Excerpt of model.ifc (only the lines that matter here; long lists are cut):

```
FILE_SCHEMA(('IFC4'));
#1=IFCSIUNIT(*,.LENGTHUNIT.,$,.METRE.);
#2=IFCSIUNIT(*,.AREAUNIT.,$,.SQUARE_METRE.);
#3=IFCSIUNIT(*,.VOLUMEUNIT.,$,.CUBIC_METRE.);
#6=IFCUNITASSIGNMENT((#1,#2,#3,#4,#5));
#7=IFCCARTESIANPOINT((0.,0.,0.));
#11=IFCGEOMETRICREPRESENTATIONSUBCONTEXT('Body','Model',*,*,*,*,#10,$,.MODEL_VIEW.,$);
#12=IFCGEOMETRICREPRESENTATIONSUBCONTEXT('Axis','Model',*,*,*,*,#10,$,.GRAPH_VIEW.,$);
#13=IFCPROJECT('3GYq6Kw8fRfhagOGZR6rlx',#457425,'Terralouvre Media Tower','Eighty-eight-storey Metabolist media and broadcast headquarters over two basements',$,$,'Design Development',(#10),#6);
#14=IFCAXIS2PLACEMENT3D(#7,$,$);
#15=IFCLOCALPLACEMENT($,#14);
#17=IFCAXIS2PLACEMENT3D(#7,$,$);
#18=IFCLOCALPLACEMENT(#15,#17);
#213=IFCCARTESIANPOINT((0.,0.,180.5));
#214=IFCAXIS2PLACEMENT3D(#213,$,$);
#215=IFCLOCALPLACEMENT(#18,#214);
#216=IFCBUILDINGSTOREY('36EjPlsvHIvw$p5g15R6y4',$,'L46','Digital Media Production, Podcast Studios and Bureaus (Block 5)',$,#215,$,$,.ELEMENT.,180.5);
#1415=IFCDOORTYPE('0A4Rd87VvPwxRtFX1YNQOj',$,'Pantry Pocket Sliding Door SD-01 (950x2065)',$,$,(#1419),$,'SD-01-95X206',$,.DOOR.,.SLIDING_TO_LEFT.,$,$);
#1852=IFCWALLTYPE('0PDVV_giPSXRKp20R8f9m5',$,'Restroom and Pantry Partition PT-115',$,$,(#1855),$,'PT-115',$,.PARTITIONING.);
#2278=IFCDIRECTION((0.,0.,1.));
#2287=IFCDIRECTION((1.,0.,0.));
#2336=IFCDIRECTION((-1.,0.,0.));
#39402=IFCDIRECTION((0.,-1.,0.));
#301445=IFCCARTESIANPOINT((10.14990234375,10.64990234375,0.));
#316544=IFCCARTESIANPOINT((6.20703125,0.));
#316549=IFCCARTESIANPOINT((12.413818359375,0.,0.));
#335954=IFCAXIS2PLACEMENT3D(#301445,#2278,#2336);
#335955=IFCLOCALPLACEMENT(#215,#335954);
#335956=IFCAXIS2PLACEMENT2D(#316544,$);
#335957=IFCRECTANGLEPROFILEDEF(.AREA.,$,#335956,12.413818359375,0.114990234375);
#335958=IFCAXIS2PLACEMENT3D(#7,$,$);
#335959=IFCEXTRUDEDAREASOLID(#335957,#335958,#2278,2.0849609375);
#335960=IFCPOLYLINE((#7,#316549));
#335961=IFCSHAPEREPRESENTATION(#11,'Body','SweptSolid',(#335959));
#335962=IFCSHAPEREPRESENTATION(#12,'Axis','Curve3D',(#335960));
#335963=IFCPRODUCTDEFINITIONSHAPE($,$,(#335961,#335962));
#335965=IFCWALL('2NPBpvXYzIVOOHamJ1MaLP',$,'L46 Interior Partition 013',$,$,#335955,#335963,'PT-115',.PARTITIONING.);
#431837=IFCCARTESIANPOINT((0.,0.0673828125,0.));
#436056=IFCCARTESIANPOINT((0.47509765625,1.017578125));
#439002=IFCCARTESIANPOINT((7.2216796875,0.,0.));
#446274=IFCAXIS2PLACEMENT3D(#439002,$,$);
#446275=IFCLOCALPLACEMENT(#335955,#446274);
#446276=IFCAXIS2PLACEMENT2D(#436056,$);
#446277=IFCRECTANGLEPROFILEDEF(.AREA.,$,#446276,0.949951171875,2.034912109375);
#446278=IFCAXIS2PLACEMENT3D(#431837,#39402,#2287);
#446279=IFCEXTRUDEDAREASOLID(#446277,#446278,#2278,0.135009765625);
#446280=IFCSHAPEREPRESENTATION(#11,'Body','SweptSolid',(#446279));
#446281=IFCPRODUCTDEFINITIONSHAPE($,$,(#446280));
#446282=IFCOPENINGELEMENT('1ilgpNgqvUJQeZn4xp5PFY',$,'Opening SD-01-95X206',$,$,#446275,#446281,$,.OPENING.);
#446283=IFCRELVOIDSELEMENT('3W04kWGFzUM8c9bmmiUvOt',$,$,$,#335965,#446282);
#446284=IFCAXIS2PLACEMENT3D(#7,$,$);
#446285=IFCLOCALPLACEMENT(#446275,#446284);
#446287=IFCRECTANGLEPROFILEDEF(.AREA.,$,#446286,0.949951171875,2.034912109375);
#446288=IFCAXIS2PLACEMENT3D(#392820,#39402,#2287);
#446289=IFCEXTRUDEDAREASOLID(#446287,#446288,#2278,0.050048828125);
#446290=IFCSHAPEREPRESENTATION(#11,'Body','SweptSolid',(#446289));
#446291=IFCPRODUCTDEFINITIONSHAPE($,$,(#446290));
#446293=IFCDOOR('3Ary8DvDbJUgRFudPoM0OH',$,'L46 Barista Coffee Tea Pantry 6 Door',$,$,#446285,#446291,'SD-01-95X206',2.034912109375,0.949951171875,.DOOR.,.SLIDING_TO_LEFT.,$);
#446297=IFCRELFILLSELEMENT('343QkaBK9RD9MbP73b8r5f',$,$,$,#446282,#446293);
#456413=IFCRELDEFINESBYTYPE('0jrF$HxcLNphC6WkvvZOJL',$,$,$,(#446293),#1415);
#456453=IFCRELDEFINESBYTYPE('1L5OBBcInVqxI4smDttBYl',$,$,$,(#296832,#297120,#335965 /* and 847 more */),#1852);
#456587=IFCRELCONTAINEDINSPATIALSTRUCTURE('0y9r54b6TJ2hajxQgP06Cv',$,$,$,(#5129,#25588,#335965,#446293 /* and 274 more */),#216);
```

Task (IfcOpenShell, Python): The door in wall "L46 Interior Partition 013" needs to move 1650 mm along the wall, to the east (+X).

```python
import ifcopenshell
import ifcopenshell.api.geometry
import ifcopenshell.util.placement
import ifcopenshell.util.unit

model = ifcopenshell.open("model.ifc")
unit_scale = ifcopenshell.util.unit.calculate_unit_scale(model)

door = model.by_id(446293)
opening = door.FillsVoids[0].RelatingOpeningElement
wall = opening.VoidsElements[0].RelatingBuildingElement

wall_matrix = ifcopenshell.util.placement.get_local_placement(wall.ObjectPlacement)
shift = wall_matrix[:3, 0] * -1.65 / unit_scale
before = ifcopenshell.util.placement.get_local_placement(door.ObjectPlacement)[:3, 3].copy()

# The door is placed relative to its opening, so it follows when the opening moves.
matrix = ifcopenshell.util.placement.get_local_placement(opening.ObjectPlacement)
matrix[:3, 3] += shift
ifcopenshell.api.geometry.edit_object_placement(
    model, product=opening, matrix=matrix, is_si=False, should_transform_children=True
)

after = ifcopenshell.util.placement.get_local_placement(door.ObjectPlacement)[:3, 3]
print("door moved by", (after - before).round(3) + 0.0)

model.write("model_edited.ifc")
```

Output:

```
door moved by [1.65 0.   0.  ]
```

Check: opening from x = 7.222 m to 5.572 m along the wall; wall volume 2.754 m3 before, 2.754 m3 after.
